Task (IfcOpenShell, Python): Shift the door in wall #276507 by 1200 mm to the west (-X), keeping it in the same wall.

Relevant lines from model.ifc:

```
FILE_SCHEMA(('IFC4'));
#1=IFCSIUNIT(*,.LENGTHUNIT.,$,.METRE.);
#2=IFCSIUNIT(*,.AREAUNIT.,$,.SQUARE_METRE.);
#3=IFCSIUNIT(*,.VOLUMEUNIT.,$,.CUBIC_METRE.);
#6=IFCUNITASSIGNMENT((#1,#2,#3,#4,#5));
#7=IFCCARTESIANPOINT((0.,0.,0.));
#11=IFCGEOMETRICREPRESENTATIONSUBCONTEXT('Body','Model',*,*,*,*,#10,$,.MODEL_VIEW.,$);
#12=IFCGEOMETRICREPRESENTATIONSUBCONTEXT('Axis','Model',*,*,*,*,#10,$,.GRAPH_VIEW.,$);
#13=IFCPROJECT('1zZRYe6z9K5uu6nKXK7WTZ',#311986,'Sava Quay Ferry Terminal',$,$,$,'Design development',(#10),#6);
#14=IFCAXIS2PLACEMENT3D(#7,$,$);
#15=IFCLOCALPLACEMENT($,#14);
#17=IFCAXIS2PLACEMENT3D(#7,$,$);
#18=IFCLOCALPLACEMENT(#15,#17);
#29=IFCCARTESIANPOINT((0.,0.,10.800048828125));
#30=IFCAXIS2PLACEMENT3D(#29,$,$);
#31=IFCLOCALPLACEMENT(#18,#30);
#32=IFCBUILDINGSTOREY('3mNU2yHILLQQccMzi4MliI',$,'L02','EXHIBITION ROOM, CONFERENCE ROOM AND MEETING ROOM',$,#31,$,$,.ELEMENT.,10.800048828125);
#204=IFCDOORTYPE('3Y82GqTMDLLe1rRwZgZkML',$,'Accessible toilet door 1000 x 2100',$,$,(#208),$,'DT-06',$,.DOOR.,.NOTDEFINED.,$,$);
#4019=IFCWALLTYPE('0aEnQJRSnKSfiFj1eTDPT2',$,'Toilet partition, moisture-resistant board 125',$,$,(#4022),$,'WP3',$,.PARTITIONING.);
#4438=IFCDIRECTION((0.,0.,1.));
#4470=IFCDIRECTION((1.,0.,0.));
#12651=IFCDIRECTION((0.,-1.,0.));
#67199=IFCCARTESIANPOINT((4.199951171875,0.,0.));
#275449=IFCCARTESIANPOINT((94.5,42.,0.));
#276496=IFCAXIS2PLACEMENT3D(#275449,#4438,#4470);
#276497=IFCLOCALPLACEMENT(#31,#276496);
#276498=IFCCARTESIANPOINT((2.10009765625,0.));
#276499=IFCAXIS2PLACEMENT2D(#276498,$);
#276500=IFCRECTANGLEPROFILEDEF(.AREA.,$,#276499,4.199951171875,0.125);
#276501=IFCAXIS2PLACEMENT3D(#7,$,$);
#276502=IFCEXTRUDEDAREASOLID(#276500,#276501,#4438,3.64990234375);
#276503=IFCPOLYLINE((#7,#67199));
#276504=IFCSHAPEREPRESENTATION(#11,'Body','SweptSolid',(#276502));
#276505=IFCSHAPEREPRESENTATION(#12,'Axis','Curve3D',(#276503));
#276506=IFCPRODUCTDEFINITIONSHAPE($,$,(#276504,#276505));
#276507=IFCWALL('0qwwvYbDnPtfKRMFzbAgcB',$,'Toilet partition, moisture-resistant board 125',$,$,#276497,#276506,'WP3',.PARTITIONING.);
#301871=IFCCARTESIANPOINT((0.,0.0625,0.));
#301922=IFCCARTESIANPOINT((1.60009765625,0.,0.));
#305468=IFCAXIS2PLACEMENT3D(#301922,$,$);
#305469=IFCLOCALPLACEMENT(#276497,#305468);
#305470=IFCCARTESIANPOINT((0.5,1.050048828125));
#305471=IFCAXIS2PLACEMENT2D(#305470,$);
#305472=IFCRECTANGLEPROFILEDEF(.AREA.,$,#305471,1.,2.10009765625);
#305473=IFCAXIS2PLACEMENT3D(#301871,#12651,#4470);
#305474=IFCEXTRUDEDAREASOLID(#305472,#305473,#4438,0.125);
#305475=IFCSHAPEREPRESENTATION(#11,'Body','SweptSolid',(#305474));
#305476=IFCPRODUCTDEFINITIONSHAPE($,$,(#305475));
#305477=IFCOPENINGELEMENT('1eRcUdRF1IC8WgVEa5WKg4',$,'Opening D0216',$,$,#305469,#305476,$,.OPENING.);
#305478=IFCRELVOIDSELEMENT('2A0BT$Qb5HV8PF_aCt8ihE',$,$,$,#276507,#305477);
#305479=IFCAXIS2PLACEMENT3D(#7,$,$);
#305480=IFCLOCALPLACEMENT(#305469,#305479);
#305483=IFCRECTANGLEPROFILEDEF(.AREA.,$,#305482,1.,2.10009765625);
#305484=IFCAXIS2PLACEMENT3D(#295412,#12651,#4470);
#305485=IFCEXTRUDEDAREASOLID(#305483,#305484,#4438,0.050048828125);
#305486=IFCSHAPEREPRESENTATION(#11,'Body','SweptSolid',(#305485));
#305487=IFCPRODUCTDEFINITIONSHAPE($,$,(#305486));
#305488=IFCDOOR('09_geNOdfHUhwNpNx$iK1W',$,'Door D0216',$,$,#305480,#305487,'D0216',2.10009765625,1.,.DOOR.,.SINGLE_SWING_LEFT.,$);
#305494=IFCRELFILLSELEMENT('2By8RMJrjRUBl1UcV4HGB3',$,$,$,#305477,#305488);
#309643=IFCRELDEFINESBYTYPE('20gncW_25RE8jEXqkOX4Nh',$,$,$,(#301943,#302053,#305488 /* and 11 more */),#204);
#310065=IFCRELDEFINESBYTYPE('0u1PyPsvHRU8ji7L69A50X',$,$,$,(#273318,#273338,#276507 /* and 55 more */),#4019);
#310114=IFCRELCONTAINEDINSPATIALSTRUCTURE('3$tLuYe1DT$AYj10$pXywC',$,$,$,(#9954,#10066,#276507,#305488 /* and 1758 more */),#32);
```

```python
import ifcopenshell
import ifcopenshell.api.geometry
import ifcopenshell.util.placement
import ifcopenshell.util.unit

model = ifcopenshell.open("model.ifc")
unit_scale = ifcopenshell.util.unit.calculate_unit_scale(model)

door = model.by_guid("09_geNOdfHUhwNpNx$iK1W")
opening = door.FillsVoids[0].RelatingOpeningElement
wall = opening.VoidsElements[0].RelatingBuildingElement

wall_matrix = ifcopenshell.util.placement.get_local_placement(wall.ObjectPlacement)
shift = wall_matrix[:3, 0] * -1.2 / unit_scale
before = ifcopenshell.util.placement.get_local_placement(door.ObjectPlacement)[:3, 3].copy()

# The door is placed relative to its opening, so it follows when the opening moves.
matrix = ifcopenshell.util.placement.get_local_placement(opening.ObjectPlacement)
matrix[:3, 3] += shift
ifcopenshell.api.geometry.edit_object_placement(
    model, product=opening, matrix=matrix, is_si=False, should_transform_children=True
)

after = ifcopenshell.util.placement.get_local_placement(door.ObjectPlacement)[:3, 3]
print("door moved by", (after - before).round(3) + 0.0)

model.write("model_rev.ifc")
```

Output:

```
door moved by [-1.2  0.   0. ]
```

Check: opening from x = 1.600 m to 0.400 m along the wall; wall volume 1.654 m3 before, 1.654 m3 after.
